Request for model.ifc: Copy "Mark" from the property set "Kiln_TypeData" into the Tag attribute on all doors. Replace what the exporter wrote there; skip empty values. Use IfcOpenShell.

First a look at what the model holds.

```python
import ifcopenshell
import ifcopenshell.util.element

model = ifcopenshell.open("model.ifc")
print(model.schema)
doors = model.by_type("IfcDoor")
print(len(doors), "doors")
for e in doors[:8]:
    source = ifcopenshell.util.element.get_pset(e, "Kiln_TypeData", "Mark")
    target = e.Tag
    print(e.id(), repr(source), repr(target), sep=" | ")
```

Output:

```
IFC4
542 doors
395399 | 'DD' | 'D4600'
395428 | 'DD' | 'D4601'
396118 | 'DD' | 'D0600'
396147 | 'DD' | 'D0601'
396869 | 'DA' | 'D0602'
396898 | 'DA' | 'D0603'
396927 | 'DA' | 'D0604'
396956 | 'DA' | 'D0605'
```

```python
import ifcopenshell
import ifcopenshell.util.element

model = ifcopenshell.open("model.ifc")

count = 0
for e in model.by_type("IfcDoor"):
    value = ifcopenshell.util.element.get_pset(e, "Kiln_TypeData", "Mark")
    current = e.Tag
    if not value or not value.strip() or current == value:
        continue
    e.Tag = value
    count += 1

print(count, "doors updated")

model.write("model_updated.ifc")
```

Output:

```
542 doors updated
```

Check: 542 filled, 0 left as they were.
